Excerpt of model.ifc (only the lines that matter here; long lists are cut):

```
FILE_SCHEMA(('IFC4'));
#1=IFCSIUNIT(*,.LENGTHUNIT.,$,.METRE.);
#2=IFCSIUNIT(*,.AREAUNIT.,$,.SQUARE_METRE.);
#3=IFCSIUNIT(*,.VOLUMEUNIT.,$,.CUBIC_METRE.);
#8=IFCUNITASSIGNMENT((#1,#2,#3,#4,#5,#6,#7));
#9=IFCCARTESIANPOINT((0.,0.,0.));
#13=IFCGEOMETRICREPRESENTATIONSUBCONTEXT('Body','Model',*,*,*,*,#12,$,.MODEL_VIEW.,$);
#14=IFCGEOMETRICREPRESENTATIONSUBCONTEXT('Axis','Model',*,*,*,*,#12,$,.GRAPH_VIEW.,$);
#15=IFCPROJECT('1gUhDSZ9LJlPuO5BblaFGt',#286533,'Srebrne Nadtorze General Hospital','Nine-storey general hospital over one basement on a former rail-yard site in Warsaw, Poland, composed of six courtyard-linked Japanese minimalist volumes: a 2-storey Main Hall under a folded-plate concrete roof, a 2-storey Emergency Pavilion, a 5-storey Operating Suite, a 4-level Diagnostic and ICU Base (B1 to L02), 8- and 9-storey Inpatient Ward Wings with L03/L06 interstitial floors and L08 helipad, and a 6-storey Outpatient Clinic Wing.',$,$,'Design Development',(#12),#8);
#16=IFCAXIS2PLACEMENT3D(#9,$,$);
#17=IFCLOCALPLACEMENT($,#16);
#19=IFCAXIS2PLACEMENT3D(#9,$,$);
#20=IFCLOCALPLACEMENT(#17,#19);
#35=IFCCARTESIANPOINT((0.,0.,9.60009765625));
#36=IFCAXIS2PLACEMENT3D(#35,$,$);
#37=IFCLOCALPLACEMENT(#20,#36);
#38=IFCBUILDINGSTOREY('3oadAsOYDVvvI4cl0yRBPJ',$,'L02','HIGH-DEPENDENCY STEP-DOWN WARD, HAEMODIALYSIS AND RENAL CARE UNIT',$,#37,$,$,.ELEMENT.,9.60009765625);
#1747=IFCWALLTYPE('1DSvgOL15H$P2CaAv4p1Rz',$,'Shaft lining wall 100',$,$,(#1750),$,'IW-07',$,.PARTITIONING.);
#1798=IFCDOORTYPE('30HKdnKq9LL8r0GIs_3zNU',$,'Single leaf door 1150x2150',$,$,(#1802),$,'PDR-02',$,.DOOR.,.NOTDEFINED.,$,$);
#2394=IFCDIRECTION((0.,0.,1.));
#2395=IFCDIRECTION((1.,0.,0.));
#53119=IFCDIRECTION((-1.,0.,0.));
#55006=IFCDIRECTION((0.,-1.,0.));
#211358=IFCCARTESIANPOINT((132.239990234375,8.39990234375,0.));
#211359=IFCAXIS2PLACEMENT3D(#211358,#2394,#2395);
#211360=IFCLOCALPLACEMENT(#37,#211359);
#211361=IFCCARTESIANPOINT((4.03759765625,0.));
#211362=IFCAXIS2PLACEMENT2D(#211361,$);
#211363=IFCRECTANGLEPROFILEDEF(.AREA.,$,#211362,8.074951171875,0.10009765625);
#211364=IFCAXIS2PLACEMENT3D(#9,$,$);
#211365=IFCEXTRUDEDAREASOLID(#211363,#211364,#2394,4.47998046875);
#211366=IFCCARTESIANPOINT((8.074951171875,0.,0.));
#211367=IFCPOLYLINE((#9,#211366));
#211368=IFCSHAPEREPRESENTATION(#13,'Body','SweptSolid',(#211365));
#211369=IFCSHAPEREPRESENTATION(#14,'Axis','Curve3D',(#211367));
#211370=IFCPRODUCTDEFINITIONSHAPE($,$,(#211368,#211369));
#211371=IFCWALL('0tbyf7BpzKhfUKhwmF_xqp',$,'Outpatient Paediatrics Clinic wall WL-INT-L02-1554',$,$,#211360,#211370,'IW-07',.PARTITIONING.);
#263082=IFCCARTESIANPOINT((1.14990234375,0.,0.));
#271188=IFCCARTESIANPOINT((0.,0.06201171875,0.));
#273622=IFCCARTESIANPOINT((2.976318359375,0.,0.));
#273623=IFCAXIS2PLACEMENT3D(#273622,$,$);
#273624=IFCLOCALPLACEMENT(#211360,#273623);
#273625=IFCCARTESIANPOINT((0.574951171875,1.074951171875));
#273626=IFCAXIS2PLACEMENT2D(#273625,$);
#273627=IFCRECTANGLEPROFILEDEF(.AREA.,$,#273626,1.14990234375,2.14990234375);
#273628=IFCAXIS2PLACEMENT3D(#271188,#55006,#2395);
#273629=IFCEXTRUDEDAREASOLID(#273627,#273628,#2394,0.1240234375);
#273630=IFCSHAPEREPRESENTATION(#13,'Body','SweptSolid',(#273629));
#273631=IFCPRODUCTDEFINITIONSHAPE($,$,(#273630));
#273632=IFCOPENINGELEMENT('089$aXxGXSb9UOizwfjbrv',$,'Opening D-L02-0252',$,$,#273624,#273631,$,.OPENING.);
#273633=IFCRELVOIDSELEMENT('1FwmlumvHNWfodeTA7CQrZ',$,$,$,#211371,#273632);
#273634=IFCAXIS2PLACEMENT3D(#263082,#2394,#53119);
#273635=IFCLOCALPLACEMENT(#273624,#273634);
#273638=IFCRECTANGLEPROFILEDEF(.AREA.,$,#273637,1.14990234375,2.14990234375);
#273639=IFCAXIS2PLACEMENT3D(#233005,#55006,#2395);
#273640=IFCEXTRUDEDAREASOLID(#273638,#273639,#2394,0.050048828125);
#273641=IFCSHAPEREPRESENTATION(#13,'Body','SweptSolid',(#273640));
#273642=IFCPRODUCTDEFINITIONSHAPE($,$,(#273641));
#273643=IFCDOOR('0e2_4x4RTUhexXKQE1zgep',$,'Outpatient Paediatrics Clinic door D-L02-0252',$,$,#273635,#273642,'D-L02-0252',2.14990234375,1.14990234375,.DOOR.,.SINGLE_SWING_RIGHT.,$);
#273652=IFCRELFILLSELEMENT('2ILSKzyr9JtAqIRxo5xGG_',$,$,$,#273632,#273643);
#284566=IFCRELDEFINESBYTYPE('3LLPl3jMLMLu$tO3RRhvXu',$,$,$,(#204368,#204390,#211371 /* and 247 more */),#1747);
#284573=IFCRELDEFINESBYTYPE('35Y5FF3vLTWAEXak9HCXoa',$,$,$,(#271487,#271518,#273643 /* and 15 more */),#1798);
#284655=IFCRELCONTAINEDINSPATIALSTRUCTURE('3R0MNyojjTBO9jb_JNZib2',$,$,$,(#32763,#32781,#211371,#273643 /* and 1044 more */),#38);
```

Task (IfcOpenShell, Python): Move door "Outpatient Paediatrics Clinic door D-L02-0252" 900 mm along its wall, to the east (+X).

```python
import ifcopenshell
import ifcopenshell.api.geometry
import ifcopenshell.util.placement

model = ifcopenshell.open("model.ifc")

door = model.by_guid("0e2_4x4RTUhexXKQE1zgep")
opening = door.FillsVoids[0].RelatingOpeningElement
wall = opening.VoidsElements[0].RelatingBuildingElement

wall_matrix = ifcopenshell.util.placement.get_local_placement(wall.ObjectPlacement)
shift = wall_matrix[:3, 0] * 0.9
before = ifcopenshell.util.placement.get_local_placement(door.ObjectPlacement)[:3, 3].copy()

# The door is placed relative to its opening, so it follows when the opening moves.
matrix = ifcopenshell.util.placement.get_local_placement(opening.ObjectPlacement)
matrix[:3, 3] += shift
ifcopenshell.api.geometry.edit_object_placement(
    model, product=opening, matrix=matrix, is_si=False, should_transform_children=True
)

after = ifcopenshell.util.placement.get_local_placement(door.ObjectPlacement)[:3, 3]
print("door moved by", (after - before).round(3) + 0.0)

model.write("model_updated.ifc")
```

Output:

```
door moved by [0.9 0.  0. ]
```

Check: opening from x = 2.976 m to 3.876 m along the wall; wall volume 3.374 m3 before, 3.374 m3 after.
